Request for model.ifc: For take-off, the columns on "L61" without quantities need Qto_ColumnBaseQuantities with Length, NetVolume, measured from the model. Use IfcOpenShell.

First a look at what the model holds.

```python
import ifcopenshell
import ifcopenshell.util.element
import ifcopenshell.util.unit

model = ifcopenshell.open("model.ifc")
print(model.schema)
for unit_type in ("LENGTHUNIT", "AREAUNIT", "VOLUMEUNIT"):
    print(unit_type, ifcopenshell.util.unit.calculate_unit_scale(model, unit_type))
storey = next(s for s in model.by_type("IfcBuildingStorey") if s.Name == "L61")
columns = [e for e in ifcopenshell.util.element.get_decomposition(storey) if e.is_a("IfcColumn")]
for e in sorted(columns, key=lambda e: e.id()):
    print(e.id(), e.is_a(), e.Name, list(ifcopenshell.util.element.get_psets(e, qtos_only=True)), sep=" | ")
```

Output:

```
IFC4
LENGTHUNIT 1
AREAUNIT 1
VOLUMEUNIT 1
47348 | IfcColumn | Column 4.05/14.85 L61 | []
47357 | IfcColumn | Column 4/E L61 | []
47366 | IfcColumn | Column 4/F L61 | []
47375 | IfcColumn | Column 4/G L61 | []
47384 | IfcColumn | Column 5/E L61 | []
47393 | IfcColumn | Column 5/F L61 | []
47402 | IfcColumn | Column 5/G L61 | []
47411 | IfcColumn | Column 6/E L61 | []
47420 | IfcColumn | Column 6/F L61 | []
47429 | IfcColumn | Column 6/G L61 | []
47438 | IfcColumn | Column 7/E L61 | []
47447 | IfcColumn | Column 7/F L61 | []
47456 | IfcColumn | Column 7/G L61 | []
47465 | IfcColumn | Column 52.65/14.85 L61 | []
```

```python
import ifcopenshell
import ifcopenshell.api.pset
import ifcopenshell.geom
import ifcopenshell.util.element
import ifcopenshell.util.shape
import ifcopenshell.util.unit

model = ifcopenshell.open("model.ifc")
unit_scale = ifcopenshell.util.unit.calculate_unit_scale(model)
volume_scale = ifcopenshell.util.unit.calculate_unit_scale(model, "VOLUMEUNIT")
settings = ifcopenshell.geom.settings()

storey = next(s for s in model.by_type("IfcBuildingStorey") if s.Name == "L61")
columns = [e for e in ifcopenshell.util.element.get_decomposition(storey) if e.is_a("IfcColumn")]

for e in sorted(columns, key=lambda e: e.id()):
    if ifcopenshell.util.element.get_psets(e, qtos_only=True, should_inherit=False):
        continue
    # Geometry comes back in metres, in the element's own axes.
    shape = ifcopenshell.geom.create_shape(settings, e)
    values = {
        "Length": ifcopenshell.util.shape.get_z(shape.geometry) / unit_scale,
        "NetVolume": ifcopenshell.util.shape.get_volume(shape.geometry) / volume_scale,
    }
    qto = ifcopenshell.api.pset.add_qto(model, product=e, name="Qto_ColumnBaseQuantities")
    ifcopenshell.api.pset.edit_qto(model, qto=qto, properties=values)
    print(e.id(), {k: round(v, 3) for k, v in values.items()})

model.write("model_edited.ifc")
```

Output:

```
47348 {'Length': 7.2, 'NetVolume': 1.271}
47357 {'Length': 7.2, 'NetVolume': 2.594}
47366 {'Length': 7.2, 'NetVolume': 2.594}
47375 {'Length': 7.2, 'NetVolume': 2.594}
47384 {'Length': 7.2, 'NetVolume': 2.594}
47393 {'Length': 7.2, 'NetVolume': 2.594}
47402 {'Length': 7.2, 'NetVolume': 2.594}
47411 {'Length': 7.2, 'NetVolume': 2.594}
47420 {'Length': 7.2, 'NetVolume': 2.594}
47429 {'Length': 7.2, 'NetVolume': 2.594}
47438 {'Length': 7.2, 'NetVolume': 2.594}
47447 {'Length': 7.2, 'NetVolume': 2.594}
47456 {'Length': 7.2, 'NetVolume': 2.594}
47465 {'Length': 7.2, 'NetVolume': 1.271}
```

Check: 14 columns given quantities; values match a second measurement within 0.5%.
